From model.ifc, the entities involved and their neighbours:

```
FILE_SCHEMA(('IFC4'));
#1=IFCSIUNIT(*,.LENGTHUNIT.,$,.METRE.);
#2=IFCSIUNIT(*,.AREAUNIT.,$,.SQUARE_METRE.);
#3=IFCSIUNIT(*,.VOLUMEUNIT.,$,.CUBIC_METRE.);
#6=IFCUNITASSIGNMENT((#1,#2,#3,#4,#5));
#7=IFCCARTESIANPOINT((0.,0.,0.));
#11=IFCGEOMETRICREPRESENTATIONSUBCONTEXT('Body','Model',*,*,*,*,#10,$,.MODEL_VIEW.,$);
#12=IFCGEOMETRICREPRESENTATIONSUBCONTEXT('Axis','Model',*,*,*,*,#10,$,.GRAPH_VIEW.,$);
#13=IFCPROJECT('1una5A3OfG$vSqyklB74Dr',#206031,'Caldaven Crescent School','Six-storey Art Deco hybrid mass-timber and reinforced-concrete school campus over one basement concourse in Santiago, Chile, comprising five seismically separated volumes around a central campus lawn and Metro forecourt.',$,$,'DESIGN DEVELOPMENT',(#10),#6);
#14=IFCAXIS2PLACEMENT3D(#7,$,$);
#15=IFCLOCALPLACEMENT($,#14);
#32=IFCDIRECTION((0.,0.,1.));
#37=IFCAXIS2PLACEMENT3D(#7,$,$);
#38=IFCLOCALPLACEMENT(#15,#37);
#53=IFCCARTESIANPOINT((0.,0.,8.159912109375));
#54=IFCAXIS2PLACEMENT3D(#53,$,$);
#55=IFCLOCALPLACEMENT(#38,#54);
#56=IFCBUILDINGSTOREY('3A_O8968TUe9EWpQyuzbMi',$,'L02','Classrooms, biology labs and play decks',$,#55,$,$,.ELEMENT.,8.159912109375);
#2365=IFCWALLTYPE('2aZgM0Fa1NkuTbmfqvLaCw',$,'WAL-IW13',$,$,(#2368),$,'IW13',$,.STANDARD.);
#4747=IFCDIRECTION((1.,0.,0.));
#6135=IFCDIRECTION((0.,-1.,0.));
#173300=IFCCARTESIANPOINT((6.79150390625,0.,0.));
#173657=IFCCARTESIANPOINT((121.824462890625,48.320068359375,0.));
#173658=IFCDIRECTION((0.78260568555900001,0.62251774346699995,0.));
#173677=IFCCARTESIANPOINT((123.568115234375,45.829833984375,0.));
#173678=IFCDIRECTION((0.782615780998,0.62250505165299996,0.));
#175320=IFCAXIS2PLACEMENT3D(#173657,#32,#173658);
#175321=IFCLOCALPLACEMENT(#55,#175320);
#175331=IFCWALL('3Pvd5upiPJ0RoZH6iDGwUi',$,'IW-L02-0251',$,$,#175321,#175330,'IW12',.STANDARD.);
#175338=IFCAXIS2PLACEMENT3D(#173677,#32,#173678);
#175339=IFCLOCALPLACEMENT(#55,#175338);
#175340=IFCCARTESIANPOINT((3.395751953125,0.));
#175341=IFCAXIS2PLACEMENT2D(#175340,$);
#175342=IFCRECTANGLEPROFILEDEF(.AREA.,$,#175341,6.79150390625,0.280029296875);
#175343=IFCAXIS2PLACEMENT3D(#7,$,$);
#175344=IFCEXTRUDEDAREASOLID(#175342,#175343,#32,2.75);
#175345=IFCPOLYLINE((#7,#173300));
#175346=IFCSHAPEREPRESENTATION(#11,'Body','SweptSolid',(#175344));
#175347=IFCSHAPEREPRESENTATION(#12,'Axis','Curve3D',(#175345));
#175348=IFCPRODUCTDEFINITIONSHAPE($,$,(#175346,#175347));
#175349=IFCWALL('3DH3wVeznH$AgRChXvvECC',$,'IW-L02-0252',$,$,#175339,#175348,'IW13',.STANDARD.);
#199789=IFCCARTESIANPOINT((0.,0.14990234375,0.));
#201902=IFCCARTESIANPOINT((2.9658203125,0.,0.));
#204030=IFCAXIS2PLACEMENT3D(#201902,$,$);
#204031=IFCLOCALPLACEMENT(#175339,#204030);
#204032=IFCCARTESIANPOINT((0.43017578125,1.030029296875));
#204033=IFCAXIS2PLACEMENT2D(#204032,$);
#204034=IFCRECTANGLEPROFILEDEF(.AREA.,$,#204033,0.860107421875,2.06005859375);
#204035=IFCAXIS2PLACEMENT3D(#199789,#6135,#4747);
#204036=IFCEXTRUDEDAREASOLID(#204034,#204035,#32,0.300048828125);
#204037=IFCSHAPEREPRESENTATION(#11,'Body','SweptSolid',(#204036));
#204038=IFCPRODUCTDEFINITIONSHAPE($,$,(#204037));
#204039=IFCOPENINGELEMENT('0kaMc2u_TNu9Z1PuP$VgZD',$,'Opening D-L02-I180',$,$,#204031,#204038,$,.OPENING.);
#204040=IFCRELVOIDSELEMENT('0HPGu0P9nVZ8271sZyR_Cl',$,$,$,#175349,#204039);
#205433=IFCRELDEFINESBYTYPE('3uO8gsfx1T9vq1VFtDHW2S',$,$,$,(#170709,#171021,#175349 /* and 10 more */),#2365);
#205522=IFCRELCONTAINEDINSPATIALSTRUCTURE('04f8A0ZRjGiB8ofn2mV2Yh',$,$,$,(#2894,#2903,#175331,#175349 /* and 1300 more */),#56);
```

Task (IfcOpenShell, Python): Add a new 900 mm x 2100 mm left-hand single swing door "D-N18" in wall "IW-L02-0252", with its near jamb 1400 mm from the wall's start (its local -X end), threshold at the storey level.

```python
import numpy as np
import ifcopenshell
import ifcopenshell.api.feature
import ifcopenshell.api.geometry
import ifcopenshell.api.root
import ifcopenshell.api.spatial
import ifcopenshell.geom
import ifcopenshell.util.element
import ifcopenshell.util.placement
import ifcopenshell.util.representation
import ifcopenshell.util.shape
import ifcopenshell.util.unit

model = ifcopenshell.open("model.ifc")
unit_scale = ifcopenshell.util.unit.calculate_unit_scale(model)
settings = ifcopenshell.geom.settings()


def volume(element):
    """Net volume in cubic metres, openings subtracted."""
    shape = ifcopenshell.geom.create_shape(settings, element)
    return ifcopenshell.util.shape.get_volume(shape.geometry)


wall = model.by_id(175349)
storey = ifcopenshell.util.element.get_container(wall, ifc_class="IfcBuildingStorey")
context = ifcopenshell.util.representation.get_context(model, "Model", "Body", "MODEL_VIEW")
before = volume(wall)

width, height, from_end, sill = 0.9, 2.1, 1.4, 0.0  # metres

# The wall runs along its own X axis, and the end named is its -X end.
wall_shape = ifcopenshell.geom.create_shape(settings, wall)
x, y, z = ifcopenshell.util.shape.get_vertices(wall_shape.geometry).T
start = x.min() + from_end
face, thickness = float(y.min()), float(y.max() - y.min())
wall_matrix = ifcopenshell.util.placement.get_local_placement(wall.ObjectPlacement)
level = ifcopenshell.util.placement.get_local_placement(storey.ObjectPlacement)[2, 3]


def in_wall(x, y):
    """Placement at x, y metres in the wall's axes, at sill height."""
    matrix = wall_matrix.copy()
    matrix[:, 3] = wall_matrix @ np.array([x / unit_scale, y / unit_scale, 0.0, 1.0])
    matrix[2, 3] = level + sill / unit_scale
    return matrix


# Opening: a box that overshoots both wall faces by 50 mm.
opening = ifcopenshell.api.root.create_entity(model, ifc_class="IfcOpeningElement", predefined_type="OPENING")
box = ifcopenshell.api.geometry.add_wall_representation(
    model, context=context, length=width, height=height, thickness=thickness + 0.1
)
ifcopenshell.api.geometry.assign_representation(model, product=opening, representation=box)
ifcopenshell.api.geometry.edit_object_placement(model, product=opening, matrix=in_wall(start, face - 0.05), is_si=False)
ifcopenshell.api.feature.add_feature(model, feature=opening, element=wall)

door = ifcopenshell.api.root.create_entity(model, ifc_class="IfcDoor", name="D-N18", predefined_type="DOOR")
door.OverallWidth, door.OverallHeight = width / unit_scale, height / unit_scale
door.OperationType = "SINGLE_SWING_LEFT"
body = ifcopenshell.api.geometry.add_door_representation(
    model,
    context=context,
    overall_width=door.OverallWidth,
    overall_height=door.OverallHeight,
    operation_type="SINGLE_SWING_LEFT",
    lining_properties={"LiningDepth": thickness / unit_scale, "ThresholdDepth": thickness / unit_scale},
)
ifcopenshell.api.geometry.assign_representation(model, product=door, representation=body)
ifcopenshell.api.spatial.assign_container(model, products=[door], relating_structure=storey)
ifcopenshell.api.feature.add_filling(model, opening=opening, element=door)

# The lining spans the wall, so the door starts at the wall face.
ifcopenshell.api.geometry.edit_object_placement(model, product=door, matrix=in_wall(start, face), is_si=False)

after = volume(wall)

print(f"wall volume {before:.3f} -> {after:.3f} m3")

model.write("model_updated.ifc")
```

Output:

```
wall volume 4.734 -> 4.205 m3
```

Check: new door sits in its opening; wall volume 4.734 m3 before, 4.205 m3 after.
